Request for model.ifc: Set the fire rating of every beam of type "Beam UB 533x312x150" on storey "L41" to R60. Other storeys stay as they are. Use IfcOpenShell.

First a look at what the model holds.

```python
import ifcopenshell
import ifcopenshell.util.element

model = ifcopenshell.open("model.ifc")
print(model.schema)
storey = next(s for s in model.by_type("IfcBuildingStorey") if s.Name == "L41")
beams = [e for e in ifcopenshell.util.element.get_decomposition(storey) if e.is_a("IfcBeam")]
seen = {}
for e in beams:
    element_type = ifcopenshell.util.element.get_type(e)
    key = (element_type.Name if element_type != e and element_type else None, ifcopenshell.util.element.get_pset(e, "Pset_BeamCommon", "FireRating"))
    seen[key] = seen.get(key, 0) + 1
for (name, value), count in sorted(seen.items(), key=str):
    print(count, "x", name, "|", value)
```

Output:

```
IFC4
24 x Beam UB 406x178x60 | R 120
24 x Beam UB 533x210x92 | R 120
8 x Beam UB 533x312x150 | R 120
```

```python
import ifcopenshell
import ifcopenshell.api.pset
import ifcopenshell.util.element

model = ifcopenshell.open("model.ifc")

storey = next(s for s in model.by_type("IfcBuildingStorey") if s.Name == "L41")
beams = [e for e in ifcopenshell.util.element.get_decomposition(storey) if e.is_a("IfcBeam")]

count = 0
for e in beams:
    element_type = ifcopenshell.util.element.get_type(e)
    if element_type in (None, e) or element_type.Name != "Beam UB 533x312x150":
        continue
    found = ifcopenshell.util.element.get_pset(e, "Pset_BeamCommon", should_inherit=False)
    if found:
        pset = model.by_id(found["id"])
        if len(ifcopenshell.util.element.get_elements_by_pset(pset)) > 1:
            pset = ifcopenshell.api.pset.unshare_pset(model, products=[e], pset=pset)[0]
    else:
        pset = ifcopenshell.api.pset.add_pset(model, product=e, name="Pset_BeamCommon")
    ifcopenshell.api.pset.edit_pset(model, pset=pset, properties={"FireRating": "R60"})
    count += 1

print(count, "beams updated")

model.write("model-out.ifc")
```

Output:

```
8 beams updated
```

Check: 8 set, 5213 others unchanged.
